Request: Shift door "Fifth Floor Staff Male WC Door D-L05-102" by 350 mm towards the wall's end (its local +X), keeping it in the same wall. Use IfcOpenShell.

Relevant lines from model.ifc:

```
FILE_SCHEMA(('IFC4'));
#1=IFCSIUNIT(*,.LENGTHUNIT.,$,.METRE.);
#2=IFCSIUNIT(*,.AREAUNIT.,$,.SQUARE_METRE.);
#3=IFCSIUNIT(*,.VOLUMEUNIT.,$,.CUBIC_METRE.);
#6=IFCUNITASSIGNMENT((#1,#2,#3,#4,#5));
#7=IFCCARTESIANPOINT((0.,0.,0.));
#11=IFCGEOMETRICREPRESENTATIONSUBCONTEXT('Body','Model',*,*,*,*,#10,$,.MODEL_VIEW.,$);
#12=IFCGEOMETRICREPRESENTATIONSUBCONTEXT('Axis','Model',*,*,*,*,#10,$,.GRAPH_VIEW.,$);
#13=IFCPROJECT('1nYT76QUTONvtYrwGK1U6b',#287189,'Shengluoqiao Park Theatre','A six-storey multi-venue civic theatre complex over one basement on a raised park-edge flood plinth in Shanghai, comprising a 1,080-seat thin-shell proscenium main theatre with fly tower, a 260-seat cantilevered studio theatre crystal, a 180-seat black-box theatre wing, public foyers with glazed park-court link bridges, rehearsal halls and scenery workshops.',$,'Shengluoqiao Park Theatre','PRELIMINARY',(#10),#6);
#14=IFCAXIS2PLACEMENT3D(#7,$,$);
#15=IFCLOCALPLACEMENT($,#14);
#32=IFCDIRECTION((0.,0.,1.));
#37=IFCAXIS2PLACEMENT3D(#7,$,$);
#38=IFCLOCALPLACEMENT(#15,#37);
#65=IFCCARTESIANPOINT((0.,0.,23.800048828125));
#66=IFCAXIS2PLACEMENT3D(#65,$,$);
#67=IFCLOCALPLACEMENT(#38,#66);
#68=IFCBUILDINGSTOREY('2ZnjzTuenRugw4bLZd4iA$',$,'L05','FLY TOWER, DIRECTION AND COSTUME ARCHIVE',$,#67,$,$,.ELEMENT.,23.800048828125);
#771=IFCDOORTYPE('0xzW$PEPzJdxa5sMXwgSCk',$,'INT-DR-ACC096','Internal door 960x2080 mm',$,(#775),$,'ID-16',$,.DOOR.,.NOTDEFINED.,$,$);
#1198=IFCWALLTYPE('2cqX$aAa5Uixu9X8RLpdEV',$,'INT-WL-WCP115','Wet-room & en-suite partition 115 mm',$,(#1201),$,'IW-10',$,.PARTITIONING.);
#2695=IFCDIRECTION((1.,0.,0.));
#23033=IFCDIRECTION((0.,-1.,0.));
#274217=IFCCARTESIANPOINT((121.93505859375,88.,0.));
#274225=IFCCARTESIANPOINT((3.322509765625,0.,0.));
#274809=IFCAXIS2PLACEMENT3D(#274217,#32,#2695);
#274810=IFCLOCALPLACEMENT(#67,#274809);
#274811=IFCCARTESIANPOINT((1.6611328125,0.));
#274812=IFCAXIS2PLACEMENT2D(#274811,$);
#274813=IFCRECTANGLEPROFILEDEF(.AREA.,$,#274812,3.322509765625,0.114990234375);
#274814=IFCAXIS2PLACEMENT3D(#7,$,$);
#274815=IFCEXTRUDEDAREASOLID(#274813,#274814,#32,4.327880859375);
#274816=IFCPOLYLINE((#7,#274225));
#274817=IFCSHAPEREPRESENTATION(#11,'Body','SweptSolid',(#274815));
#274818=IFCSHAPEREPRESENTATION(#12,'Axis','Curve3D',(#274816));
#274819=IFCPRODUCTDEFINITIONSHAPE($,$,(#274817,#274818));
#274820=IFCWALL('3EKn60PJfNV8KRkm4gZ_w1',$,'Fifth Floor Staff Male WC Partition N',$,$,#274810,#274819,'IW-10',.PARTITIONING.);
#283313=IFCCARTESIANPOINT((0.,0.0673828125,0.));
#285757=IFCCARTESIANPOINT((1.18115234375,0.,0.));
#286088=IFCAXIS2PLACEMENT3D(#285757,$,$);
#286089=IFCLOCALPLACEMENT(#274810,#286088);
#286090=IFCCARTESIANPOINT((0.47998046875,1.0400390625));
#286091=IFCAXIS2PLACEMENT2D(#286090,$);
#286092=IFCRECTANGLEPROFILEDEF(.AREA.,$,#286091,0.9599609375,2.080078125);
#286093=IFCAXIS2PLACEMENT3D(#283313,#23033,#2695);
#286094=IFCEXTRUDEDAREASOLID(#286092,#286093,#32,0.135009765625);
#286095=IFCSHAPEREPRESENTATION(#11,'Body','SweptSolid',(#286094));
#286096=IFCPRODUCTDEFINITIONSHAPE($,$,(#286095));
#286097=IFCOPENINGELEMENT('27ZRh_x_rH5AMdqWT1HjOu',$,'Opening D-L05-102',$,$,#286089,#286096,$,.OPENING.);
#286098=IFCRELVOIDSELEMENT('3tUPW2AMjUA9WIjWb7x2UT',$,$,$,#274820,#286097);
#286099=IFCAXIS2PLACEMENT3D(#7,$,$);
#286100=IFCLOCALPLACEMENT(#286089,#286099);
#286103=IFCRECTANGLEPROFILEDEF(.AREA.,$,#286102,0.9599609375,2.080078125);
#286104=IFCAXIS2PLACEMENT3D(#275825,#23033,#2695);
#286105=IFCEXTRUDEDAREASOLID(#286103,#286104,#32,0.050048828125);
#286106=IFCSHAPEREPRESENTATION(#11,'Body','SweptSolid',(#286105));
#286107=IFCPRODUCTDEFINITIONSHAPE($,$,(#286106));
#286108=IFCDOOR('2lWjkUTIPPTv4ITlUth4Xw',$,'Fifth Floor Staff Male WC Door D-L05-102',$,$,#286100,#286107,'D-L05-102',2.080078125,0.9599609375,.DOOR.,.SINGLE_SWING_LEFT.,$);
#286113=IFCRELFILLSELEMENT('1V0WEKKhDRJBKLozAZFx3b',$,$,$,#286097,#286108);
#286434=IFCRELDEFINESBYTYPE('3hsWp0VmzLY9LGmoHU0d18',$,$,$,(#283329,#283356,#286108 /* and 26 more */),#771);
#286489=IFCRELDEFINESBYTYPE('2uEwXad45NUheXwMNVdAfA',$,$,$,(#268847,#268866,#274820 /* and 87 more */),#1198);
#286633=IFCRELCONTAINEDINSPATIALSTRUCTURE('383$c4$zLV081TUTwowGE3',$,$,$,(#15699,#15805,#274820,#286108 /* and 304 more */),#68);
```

```python
import ifcopenshell
import ifcopenshell.api.geometry
import ifcopenshell.util.placement
import ifcopenshell.util.unit

model = ifcopenshell.open("model.ifc")
unit_scale = ifcopenshell.util.unit.calculate_unit_scale(model)

door = model.by_guid("2lWjkUTIPPTv4ITlUth4Xw")
opening = door.FillsVoids[0].RelatingOpeningElement
wall = opening.VoidsElements[0].RelatingBuildingElement

wall_matrix = ifcopenshell.util.placement.get_local_placement(wall.ObjectPlacement)
shift = wall_matrix[:3, 0] * 0.35 / unit_scale
before = ifcopenshell.util.placement.get_local_placement(door.ObjectPlacement)[:3, 3].copy()

# The door is placed relative to its opening, so it follows when the opening moves.
matrix = ifcopenshell.util.placement.get_local_placement(opening.ObjectPlacement)
matrix[:3, 3] += shift
ifcopenshell.api.geometry.edit_object_placement(
    model, product=opening, matrix=matrix, is_si=False, should_transform_children=True
)

after = ifcopenshell.util.placement.get_local_placement(door.ObjectPlacement)[:3, 3]
print("door moved by", (after - before).round(3) + 0.0)

model.write("model_rev.ifc")
```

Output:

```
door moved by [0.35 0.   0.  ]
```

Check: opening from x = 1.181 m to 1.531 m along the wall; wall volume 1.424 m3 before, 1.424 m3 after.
